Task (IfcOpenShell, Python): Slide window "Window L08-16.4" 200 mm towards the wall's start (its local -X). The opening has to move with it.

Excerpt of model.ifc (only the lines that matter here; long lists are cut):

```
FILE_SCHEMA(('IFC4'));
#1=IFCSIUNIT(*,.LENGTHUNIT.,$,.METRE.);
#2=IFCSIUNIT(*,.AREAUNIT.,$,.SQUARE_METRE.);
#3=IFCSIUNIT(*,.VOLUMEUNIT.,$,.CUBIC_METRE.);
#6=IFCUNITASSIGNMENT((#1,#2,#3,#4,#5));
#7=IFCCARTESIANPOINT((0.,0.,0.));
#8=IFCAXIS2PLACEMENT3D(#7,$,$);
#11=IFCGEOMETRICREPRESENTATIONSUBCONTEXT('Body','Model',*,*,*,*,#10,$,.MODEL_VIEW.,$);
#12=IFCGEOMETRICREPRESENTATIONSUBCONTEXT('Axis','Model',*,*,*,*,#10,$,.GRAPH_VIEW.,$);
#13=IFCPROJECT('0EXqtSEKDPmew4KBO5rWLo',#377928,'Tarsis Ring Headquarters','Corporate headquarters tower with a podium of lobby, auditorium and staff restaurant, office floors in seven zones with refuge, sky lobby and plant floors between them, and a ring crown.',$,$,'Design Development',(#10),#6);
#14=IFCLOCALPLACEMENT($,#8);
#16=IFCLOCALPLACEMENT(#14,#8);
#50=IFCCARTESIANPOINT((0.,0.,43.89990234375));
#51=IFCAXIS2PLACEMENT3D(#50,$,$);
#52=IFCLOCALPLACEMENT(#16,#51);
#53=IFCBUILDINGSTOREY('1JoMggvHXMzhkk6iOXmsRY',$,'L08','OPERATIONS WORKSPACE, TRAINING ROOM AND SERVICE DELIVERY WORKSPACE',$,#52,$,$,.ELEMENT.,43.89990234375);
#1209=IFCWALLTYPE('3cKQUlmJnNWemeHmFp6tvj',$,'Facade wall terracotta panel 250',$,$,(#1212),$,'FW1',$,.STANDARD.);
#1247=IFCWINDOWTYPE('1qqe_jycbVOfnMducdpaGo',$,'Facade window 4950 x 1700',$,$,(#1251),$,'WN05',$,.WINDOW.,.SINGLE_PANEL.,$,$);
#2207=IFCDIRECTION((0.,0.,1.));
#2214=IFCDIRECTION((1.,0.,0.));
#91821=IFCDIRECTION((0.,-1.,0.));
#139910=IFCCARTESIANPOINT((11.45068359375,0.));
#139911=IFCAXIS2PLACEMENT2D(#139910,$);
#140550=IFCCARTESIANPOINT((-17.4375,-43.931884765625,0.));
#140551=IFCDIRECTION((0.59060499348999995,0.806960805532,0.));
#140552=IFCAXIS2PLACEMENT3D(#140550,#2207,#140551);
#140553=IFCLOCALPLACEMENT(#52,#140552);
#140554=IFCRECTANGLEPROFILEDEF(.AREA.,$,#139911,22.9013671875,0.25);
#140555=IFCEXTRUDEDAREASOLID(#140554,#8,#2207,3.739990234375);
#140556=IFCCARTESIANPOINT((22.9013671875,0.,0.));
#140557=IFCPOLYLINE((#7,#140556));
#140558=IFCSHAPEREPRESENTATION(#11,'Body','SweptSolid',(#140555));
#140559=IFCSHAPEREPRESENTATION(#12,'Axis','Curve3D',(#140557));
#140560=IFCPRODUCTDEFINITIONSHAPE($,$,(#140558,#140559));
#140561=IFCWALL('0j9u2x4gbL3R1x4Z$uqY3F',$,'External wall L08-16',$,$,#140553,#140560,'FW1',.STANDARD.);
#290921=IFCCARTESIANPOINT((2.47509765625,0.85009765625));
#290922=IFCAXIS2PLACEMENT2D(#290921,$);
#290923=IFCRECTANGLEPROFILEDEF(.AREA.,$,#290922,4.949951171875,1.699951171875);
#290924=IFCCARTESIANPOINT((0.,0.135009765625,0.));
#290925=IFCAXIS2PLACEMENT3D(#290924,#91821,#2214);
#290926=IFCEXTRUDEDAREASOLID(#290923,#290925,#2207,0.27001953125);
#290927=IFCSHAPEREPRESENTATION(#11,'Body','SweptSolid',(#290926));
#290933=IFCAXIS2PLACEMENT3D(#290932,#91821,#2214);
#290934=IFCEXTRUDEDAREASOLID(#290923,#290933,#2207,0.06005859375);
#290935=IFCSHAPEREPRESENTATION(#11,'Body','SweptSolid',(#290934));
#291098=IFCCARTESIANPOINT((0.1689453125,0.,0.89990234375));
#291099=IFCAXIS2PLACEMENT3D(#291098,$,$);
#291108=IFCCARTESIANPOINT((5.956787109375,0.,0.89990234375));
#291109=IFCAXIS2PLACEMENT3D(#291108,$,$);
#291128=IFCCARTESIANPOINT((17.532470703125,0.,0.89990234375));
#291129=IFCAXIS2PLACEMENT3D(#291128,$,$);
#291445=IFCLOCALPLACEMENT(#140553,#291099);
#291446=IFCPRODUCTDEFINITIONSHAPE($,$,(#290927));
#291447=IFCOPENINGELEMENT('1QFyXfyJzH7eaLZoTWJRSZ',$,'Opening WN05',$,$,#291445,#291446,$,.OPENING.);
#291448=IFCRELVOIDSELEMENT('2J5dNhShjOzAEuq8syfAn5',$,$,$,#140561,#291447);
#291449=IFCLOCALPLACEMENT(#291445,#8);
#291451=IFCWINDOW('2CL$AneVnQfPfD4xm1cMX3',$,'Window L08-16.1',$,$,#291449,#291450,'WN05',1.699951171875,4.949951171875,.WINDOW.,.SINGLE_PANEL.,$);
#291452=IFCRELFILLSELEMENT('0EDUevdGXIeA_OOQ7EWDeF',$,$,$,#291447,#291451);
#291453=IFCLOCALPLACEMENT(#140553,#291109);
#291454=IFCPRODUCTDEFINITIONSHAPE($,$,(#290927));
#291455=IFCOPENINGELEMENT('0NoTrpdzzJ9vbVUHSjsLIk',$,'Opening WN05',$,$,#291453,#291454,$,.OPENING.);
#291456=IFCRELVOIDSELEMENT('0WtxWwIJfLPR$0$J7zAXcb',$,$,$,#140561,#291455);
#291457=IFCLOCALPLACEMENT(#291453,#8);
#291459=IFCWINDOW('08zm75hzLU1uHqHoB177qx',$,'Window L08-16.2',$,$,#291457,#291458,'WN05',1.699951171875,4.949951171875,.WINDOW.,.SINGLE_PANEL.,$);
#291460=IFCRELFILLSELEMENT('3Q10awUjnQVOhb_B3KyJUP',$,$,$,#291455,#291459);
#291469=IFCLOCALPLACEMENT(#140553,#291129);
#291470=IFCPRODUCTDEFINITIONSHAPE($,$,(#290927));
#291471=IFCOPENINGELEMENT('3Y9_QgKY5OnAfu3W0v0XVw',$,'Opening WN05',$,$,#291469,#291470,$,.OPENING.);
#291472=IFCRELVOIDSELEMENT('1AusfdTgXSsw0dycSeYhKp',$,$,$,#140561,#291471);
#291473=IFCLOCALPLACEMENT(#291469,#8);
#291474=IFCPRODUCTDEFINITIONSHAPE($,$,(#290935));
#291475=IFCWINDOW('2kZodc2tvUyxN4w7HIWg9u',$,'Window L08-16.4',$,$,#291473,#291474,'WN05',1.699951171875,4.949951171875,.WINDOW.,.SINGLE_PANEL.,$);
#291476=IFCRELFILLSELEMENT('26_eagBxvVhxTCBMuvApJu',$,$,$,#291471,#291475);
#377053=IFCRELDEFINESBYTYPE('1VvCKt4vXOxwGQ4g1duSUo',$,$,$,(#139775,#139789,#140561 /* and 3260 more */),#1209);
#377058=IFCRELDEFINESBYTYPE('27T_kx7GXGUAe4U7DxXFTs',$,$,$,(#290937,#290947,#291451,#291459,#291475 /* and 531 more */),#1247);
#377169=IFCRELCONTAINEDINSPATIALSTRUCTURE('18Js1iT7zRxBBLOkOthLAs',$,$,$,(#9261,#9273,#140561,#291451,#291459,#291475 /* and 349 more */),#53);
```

```python
import ifcopenshell
import ifcopenshell.api.geometry
import ifcopenshell.util.placement
import ifcopenshell.util.unit

model = ifcopenshell.open("model.ifc")
unit_scale = ifcopenshell.util.unit.calculate_unit_scale(model)

window = model.by_guid("2kZodc2tvUyxN4w7HIWg9u")
opening = window.FillsVoids[0].RelatingOpeningElement
wall = opening.VoidsElements[0].RelatingBuildingElement

wall_matrix = ifcopenshell.util.placement.get_local_placement(wall.ObjectPlacement)
shift = wall_matrix[:3, 0] * -0.2 / unit_scale
before = ifcopenshell.util.placement.get_local_placement(window.ObjectPlacement)[:3, 3].copy()

# The window is placed relative to its opening, so it follows when the opening moves.
matrix = ifcopenshell.util.placement.get_local_placement(opening.ObjectPlacement)
matrix[:3, 3] += shift
ifcopenshell.api.geometry.edit_object_placement(
    model, product=opening, matrix=matrix, is_si=False, should_transform_children=True
)

after = ifcopenshell.util.placement.get_local_placement(window.ObjectPlacement)[:3, 3]
print("window moved by", (after - before).round(3) + 0.0)

model.write("model-out.ifc")
```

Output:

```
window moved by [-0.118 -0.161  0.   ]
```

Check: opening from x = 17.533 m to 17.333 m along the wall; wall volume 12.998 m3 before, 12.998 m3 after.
